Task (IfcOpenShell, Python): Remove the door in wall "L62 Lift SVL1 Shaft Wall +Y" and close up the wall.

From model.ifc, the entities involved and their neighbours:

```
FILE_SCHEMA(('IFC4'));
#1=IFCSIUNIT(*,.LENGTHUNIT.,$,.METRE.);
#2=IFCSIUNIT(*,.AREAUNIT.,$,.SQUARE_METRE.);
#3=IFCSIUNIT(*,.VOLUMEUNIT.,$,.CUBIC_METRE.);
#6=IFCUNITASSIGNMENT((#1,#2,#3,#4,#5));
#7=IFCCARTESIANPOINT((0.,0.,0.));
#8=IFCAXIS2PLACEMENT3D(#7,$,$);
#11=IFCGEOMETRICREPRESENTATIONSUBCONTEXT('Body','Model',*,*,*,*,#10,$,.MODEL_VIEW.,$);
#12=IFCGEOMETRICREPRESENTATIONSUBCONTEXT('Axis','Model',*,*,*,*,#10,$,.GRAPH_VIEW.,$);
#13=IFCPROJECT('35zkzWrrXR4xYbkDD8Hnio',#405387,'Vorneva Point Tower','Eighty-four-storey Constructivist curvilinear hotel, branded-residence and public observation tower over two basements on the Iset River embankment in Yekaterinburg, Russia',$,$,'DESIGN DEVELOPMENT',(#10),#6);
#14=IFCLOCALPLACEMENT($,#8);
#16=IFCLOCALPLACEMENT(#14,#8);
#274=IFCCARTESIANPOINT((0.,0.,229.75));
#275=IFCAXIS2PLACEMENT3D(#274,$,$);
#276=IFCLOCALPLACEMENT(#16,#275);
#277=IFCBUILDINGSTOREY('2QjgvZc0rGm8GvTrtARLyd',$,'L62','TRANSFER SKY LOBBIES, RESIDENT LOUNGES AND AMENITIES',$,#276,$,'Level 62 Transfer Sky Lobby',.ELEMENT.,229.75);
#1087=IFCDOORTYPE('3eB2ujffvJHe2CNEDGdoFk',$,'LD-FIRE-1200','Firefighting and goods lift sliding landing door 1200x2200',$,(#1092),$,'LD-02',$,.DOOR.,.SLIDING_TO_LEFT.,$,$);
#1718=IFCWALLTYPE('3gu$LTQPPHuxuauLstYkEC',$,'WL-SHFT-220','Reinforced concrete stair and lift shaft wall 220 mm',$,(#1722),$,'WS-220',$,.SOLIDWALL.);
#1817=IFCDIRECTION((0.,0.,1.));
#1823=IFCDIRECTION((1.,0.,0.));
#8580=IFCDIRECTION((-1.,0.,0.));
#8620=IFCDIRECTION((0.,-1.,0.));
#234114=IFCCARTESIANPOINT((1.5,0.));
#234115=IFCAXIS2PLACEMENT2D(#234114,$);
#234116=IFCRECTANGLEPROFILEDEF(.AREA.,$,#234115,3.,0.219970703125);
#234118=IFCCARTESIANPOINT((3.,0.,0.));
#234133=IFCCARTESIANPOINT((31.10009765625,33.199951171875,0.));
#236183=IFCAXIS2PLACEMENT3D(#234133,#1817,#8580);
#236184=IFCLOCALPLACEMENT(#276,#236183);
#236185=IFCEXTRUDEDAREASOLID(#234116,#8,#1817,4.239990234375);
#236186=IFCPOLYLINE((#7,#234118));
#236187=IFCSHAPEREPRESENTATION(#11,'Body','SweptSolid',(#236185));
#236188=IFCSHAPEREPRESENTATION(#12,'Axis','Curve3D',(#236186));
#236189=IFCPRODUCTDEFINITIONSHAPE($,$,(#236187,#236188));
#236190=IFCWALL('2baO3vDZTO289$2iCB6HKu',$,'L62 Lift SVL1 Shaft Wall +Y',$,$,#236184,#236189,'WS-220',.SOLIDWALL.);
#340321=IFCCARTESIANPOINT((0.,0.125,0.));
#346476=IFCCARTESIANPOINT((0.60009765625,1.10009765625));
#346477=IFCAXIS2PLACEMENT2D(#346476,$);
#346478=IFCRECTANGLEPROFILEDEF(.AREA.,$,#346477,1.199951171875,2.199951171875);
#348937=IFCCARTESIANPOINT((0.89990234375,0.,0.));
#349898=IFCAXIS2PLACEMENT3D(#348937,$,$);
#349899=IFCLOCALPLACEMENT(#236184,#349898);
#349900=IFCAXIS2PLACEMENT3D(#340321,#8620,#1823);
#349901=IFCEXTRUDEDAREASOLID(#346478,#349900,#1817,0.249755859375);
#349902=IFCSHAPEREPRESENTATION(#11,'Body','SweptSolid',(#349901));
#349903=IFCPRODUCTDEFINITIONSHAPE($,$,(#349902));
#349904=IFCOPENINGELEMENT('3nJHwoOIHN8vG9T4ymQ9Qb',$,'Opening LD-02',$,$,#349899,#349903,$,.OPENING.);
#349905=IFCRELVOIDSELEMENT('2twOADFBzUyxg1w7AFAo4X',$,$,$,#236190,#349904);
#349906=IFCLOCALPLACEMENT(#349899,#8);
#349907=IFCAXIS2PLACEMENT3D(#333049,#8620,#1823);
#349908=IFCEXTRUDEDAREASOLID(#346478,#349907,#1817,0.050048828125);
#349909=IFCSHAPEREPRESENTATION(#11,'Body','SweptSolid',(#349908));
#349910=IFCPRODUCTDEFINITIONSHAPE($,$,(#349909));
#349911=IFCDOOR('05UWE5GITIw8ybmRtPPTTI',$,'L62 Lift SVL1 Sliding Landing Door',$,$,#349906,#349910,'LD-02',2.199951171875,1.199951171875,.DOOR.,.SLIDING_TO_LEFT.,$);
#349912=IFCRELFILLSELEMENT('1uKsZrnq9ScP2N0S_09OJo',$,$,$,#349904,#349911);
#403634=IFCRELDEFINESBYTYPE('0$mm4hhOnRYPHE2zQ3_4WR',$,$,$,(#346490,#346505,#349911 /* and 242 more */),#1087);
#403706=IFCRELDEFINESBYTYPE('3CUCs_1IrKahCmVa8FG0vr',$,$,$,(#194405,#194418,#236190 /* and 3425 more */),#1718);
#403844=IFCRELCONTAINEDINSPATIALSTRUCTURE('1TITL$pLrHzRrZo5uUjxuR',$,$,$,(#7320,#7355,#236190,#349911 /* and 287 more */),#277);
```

```python
import ifcopenshell
import ifcopenshell.api.feature
import ifcopenshell.api.root
import ifcopenshell.geom
import ifcopenshell.util.shape

model = ifcopenshell.open("model.ifc")
settings = ifcopenshell.geom.settings()


def volume(element):
    """Net volume in cubic metres, openings subtracted."""
    shape = ifcopenshell.geom.create_shape(settings, element)
    return ifcopenshell.util.shape.get_volume(shape.geometry)


door = model.by_guid("05UWE5GITIw8ybmRtPPTTI")
opening = door.FillsVoids[0].RelatingOpeningElement
wall = opening.VoidsElements[0].RelatingBuildingElement
before = volume(wall)

ifcopenshell.api.root.remove_product(model, product=door)
ifcopenshell.api.feature.remove_feature(model, feature=opening)

after = volume(wall)

print(f"wall volume {before:.3f} -> {after:.3f} m3")

model.write("model-out.ifc")
```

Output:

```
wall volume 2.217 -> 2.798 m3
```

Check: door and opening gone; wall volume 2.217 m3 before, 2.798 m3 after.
